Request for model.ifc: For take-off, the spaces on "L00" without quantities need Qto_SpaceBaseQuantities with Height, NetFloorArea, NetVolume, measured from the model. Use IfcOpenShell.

First a look at what the model holds.

```python
import ifcopenshell
import ifcopenshell.util.element
import ifcopenshell.util.unit

model = ifcopenshell.open("model.ifc")
print(model.schema)
for unit_type in ("LENGTHUNIT", "AREAUNIT", "VOLUMEUNIT"):
    print(unit_type, ifcopenshell.util.unit.calculate_unit_scale(model, unit_type))
storey = next(s for s in model.by_type("IfcBuildingStorey") if s.Name == "L00")
spaces = [e for e in ifcopenshell.util.element.get_decomposition(storey) if e.is_a("IfcSpace")]
for e in sorted(spaces, key=lambda e: e.id()):
    print(e.id(), e.is_a(), e.Name, list(ifcopenshell.util.element.get_psets(e, qtos_only=True)), sep=" | ")
```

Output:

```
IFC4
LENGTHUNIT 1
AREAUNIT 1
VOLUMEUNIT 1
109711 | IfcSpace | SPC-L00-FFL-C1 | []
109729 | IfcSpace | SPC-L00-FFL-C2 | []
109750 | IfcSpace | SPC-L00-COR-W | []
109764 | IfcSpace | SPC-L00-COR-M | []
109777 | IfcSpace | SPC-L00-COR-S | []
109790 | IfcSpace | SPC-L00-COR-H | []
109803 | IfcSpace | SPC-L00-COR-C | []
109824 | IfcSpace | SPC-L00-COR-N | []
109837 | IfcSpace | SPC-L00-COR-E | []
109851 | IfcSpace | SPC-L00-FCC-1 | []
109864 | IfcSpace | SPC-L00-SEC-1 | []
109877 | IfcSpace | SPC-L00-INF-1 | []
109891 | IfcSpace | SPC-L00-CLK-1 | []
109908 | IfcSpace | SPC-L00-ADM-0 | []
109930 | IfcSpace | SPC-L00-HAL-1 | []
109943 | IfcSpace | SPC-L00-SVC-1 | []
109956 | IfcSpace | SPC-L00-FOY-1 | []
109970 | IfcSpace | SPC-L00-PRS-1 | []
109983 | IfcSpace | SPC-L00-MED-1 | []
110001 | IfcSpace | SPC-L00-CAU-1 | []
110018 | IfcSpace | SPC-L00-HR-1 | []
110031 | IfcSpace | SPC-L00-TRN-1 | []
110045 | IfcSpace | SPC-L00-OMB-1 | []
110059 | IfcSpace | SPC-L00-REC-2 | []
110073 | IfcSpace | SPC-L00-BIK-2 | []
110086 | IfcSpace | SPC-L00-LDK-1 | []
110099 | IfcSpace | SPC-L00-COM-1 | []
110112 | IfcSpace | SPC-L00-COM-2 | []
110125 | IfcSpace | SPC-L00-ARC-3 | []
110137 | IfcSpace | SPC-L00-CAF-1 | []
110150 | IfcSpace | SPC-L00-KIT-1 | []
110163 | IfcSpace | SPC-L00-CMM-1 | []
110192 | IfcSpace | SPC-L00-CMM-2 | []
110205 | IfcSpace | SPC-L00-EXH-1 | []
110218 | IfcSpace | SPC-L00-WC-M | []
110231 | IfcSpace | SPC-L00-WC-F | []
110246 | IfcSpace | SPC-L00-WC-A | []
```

```python
import ifcopenshell
import ifcopenshell.api.pset
import ifcopenshell.geom
import ifcopenshell.util.element
import ifcopenshell.util.shape
import ifcopenshell.util.unit

model = ifcopenshell.open("model.ifc")
unit_scale = ifcopenshell.util.unit.calculate_unit_scale(model)
area_scale = ifcopenshell.util.unit.calculate_unit_scale(model, "AREAUNIT")
volume_scale = ifcopenshell.util.unit.calculate_unit_scale(model, "VOLUMEUNIT")
settings = ifcopenshell.geom.settings()

storey = next(s for s in model.by_type("IfcBuildingStorey") if s.Name == "L00")
spaces = [e for e in ifcopenshell.util.element.get_decomposition(storey) if e.is_a("IfcSpace")]

for e in sorted(spaces, key=lambda e: e.id()):
    if ifcopenshell.util.element.get_psets(e, qtos_only=True, should_inherit=False):
        continue
    # Geometry comes back in metres, in the element's own axes.
    shape = ifcopenshell.geom.create_shape(settings, e)
    values = {
        "Height": ifcopenshell.util.shape.get_z(shape.geometry) / unit_scale,
        "NetFloorArea": ifcopenshell.util.shape.get_footprint_area(shape.geometry) / area_scale,
        "NetVolume": ifcopenshell.util.shape.get_volume(shape.geometry) / volume_scale,
    }
    qto = ifcopenshell.api.pset.add_qto(model, product=e, name="Qto_SpaceBaseQuantities")
    ifcopenshell.api.pset.edit_qto(model, qto=qto, properties=values)
    print(e.id(), {k: round(v, 3) for k, v in values.items()})

model.write("model_rev.ifc")
```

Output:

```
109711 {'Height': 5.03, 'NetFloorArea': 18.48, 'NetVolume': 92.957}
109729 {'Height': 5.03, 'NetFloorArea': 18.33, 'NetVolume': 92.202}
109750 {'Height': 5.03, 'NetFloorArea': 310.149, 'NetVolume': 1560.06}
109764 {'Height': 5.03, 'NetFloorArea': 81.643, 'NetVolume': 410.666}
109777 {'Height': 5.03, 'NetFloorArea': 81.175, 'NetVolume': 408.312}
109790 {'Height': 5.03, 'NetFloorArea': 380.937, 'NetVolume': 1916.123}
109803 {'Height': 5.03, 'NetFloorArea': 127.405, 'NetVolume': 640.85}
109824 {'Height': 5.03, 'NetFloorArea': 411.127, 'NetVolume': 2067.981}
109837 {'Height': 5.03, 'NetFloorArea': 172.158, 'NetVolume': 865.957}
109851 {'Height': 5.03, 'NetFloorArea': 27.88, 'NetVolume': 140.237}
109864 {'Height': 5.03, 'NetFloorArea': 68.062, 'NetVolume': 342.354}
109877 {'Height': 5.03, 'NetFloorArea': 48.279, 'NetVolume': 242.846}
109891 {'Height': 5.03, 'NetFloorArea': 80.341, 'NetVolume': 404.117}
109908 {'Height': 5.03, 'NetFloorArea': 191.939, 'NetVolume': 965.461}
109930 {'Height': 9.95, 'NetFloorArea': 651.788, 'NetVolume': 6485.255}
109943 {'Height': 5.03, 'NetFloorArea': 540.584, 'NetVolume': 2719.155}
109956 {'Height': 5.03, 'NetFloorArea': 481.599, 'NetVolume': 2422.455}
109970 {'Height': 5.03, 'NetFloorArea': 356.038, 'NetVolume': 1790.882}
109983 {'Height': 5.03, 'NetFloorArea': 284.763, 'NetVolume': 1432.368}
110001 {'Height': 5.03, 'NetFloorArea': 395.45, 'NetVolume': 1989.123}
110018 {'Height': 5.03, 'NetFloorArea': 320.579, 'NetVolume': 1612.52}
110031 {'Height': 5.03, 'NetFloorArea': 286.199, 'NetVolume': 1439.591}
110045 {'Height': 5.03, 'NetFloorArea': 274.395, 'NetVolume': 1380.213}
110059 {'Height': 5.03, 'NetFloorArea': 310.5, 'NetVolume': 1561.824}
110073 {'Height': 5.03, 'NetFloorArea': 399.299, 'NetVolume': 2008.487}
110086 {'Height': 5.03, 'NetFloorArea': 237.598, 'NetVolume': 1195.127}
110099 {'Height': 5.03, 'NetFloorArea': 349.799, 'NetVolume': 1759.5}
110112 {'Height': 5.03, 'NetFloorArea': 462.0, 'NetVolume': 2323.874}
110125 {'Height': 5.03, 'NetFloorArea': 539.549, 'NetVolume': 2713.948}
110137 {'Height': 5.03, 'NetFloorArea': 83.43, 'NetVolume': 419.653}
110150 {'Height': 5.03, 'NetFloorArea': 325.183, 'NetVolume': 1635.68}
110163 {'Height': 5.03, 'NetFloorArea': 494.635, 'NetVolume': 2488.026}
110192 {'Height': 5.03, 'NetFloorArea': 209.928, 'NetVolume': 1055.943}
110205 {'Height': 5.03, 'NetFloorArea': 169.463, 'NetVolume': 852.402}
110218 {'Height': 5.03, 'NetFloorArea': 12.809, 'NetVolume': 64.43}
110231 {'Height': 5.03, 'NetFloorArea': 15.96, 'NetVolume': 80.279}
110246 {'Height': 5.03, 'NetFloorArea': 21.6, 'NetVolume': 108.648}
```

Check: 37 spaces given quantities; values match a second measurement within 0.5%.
